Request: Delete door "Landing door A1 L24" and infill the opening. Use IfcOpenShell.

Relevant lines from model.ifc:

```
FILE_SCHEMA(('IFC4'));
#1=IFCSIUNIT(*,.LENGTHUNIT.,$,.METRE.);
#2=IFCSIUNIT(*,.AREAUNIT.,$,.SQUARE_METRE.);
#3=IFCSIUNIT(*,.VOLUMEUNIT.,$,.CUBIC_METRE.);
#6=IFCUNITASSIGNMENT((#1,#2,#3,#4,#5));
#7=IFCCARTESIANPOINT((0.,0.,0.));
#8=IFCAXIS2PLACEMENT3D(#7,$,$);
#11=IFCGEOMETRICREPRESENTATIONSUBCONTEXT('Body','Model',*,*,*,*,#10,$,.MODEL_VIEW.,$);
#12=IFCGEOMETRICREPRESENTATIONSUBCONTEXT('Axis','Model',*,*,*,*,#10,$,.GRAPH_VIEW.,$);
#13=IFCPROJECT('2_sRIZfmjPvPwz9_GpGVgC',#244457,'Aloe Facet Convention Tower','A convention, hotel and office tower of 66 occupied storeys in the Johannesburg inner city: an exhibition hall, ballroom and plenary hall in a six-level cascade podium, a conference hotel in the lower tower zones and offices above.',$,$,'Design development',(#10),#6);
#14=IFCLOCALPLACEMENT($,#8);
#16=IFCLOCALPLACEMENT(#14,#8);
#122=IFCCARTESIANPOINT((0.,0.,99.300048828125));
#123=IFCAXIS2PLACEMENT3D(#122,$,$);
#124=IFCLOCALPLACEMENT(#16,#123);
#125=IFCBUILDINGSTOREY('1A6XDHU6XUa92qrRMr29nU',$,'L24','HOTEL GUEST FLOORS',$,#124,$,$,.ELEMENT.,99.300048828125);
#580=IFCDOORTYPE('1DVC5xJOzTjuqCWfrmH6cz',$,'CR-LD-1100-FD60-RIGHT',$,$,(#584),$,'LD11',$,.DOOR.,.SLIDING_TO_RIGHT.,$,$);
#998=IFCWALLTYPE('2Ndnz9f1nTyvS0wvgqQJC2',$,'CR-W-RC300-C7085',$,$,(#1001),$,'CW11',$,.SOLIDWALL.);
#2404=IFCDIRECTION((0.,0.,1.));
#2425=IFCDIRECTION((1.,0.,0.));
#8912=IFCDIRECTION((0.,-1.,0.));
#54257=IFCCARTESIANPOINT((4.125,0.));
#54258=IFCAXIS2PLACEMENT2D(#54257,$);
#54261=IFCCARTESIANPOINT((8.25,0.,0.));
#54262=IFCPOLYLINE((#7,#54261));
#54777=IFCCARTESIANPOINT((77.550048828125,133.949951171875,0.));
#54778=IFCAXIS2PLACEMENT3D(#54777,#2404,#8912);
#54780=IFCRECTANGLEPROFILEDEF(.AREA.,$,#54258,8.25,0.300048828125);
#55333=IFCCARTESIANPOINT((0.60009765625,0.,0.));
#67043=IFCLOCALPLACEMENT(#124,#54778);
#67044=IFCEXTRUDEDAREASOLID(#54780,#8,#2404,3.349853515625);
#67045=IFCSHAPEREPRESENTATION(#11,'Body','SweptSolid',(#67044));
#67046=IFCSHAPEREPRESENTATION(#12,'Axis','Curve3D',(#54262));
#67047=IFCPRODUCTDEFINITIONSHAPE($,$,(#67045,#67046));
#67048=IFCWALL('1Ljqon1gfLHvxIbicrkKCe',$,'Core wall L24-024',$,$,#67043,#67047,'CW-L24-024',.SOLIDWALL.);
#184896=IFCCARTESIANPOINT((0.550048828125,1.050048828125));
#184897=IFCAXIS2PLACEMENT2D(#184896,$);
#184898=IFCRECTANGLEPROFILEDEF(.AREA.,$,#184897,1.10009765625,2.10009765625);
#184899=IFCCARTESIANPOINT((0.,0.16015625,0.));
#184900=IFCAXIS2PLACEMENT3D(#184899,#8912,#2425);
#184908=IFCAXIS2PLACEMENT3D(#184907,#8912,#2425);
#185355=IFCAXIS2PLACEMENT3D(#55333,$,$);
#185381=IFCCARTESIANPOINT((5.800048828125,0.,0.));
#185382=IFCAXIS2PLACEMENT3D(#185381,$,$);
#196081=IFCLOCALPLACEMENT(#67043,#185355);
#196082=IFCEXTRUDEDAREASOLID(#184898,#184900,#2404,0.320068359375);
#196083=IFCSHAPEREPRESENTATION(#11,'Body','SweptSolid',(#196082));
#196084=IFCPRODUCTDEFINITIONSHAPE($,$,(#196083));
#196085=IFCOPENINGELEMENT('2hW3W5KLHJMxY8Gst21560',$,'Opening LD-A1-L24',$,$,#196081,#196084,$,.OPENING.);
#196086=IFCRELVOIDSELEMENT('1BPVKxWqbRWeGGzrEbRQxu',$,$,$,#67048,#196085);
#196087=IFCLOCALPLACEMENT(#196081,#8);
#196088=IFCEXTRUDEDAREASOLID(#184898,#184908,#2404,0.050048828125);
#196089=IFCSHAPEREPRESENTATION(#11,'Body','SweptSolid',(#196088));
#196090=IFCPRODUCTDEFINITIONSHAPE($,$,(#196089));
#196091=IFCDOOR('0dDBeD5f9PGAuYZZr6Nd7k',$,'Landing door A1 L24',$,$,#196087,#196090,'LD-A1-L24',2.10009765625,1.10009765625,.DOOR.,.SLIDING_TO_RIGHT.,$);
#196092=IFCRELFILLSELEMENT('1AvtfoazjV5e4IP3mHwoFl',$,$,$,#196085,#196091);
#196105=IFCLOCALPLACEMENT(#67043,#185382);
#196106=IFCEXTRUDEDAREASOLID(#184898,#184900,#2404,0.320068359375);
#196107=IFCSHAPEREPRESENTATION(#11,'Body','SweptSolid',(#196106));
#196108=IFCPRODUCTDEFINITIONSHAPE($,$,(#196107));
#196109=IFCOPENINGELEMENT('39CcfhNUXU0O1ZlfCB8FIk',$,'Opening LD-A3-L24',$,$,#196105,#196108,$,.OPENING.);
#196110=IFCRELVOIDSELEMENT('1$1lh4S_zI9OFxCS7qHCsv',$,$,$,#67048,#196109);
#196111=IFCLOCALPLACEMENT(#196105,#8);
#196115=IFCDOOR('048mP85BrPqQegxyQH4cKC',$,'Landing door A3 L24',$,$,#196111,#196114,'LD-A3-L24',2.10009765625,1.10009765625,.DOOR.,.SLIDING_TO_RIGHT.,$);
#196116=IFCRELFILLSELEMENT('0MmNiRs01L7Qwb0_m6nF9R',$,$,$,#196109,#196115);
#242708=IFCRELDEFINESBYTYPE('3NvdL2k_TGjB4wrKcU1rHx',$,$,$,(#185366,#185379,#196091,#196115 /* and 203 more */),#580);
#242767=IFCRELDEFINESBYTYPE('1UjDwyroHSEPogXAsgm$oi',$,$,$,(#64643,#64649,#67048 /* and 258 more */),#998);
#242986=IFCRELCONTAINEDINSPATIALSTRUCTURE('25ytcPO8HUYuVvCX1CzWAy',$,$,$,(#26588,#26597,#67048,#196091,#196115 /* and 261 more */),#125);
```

```python
import ifcopenshell
import ifcopenshell.api.feature
import ifcopenshell.api.root
import ifcopenshell.geom
import ifcopenshell.util.shape

model = ifcopenshell.open("model.ifc")
settings = ifcopenshell.geom.settings()


def volume(element):
    """Net volume in cubic metres, openings subtracted."""
    shape = ifcopenshell.geom.create_shape(settings, element)
    return ifcopenshell.util.shape.get_volume(shape.geometry)


door = model.by_guid("0dDBeD5f9PGAuYZZr6Nd7k")
opening = door.FillsVoids[0].RelatingOpeningElement
wall = opening.VoidsElements[0].RelatingBuildingElement
before = volume(wall)

ifcopenshell.api.root.remove_product(model, product=door)
ifcopenshell.api.feature.remove_feature(model, feature=opening)

after = volume(wall)

print(f"wall volume {before:.3f} -> {after:.3f} m3")

model.write("model_updated.ifc")
```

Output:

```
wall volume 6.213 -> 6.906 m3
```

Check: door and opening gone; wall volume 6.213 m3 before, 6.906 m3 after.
